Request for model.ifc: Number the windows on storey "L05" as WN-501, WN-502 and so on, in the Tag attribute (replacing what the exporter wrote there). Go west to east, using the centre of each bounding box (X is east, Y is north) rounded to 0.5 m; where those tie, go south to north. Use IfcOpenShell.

First a look at what the model holds.

```python
import ifcopenshell
import ifcopenshell.util.element
import ifcopenshell.util.placement

model = ifcopenshell.open("model.ifc")
print(model.schema)
storey = next(s for s in model.by_type("IfcBuildingStorey") if s.Name == "L05")
windows = [e for e in ifcopenshell.util.element.get_decomposition(storey) if e.is_a("IfcWindow")]
for e in sorted(windows, key=lambda e: e.id()):
    origin = ifcopenshell.util.placement.get_local_placement(e.ObjectPlacement)[:3, 3]
    print(e.id(), e.Tag, e.Name, origin.round(2) + 0.0, sep=" | ")
```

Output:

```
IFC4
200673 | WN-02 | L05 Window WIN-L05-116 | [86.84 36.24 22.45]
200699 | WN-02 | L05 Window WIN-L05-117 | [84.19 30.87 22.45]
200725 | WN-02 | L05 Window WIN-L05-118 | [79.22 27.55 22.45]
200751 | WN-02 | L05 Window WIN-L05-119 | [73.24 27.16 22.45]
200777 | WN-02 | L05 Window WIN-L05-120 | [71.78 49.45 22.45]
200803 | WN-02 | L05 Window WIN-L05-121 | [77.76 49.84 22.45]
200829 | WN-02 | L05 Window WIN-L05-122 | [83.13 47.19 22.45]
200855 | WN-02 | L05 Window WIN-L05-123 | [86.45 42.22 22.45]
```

```python
import ifcopenshell
import ifcopenshell.geom
import ifcopenshell.util.element
import ifcopenshell.util.shape

model = ifcopenshell.open("model.ifc")
settings = ifcopenshell.geom.settings()
settings.set("use-world-coords", True)


def centre(element):
    shape = ifcopenshell.geom.create_shape(settings, element)
    return ifcopenshell.util.shape.get_bbox_centroid(shape.geometry)


storey = next(s for s in model.by_type("IfcBuildingStorey") if s.Name == "L05")
windows = [e for e in ifcopenshell.util.element.get_decomposition(storey) if e.is_a("IfcWindow")]

# Insertion points can sit at a corner or the storey origin, so sort by the geometry (in metres).
centres = {e: centre(e) for e in windows}
windows.sort(key=lambda e: (round(centres[e][0] / 0.5), centres[e][1]))

for i, e in enumerate(windows, start=1):
    number = f"WN-5{i:02d}"
    e.Tag = number
    print(e.id(), number)

model.write("model_v2.ifc")
```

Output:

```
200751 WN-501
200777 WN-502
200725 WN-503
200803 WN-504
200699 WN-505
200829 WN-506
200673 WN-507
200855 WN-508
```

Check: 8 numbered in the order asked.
